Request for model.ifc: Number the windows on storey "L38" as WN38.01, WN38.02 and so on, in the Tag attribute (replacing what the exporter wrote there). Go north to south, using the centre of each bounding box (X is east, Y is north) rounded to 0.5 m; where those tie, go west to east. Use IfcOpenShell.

First a look at what the model holds.

```python
import ifcopenshell
import ifcopenshell.util.element
import ifcopenshell.util.placement

model = ifcopenshell.open("model.ifc")
print(model.schema)
storey = next(s for s in model.by_type("IfcBuildingStorey") if s.Name == "L38")
windows = [e for e in ifcopenshell.util.element.get_decomposition(storey) if e.is_a("IfcWindow")]
for e in sorted(windows, key=lambda e: e.id()):
    origin = ifcopenshell.util.placement.get_local_placement(e.ObjectPlacement)[:3, 3]
    print(e.id(), e.Tag, e.Name, origin.round(2) + 0.0, sep=" | ")
```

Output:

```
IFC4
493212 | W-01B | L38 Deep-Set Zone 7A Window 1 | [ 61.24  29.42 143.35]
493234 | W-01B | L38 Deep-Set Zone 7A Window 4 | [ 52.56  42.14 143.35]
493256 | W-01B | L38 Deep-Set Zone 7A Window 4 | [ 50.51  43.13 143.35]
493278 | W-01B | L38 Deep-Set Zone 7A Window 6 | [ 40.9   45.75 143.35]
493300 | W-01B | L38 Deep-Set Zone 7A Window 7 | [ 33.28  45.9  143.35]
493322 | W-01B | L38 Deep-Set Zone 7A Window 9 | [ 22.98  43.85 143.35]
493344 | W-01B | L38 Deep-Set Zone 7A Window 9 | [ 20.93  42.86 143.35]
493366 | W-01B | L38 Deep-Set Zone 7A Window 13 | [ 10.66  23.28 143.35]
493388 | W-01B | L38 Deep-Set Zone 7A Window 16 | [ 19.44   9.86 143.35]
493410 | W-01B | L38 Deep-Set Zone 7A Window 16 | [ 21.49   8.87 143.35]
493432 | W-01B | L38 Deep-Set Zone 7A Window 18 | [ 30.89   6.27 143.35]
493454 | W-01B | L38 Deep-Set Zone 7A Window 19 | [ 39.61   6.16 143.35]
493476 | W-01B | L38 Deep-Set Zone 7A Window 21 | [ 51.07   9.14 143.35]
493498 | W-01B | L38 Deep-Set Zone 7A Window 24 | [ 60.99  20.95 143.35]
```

```python
import ifcopenshell
import ifcopenshell.geom
import ifcopenshell.util.element
import ifcopenshell.util.shape

model = ifcopenshell.open("model.ifc")
settings = ifcopenshell.geom.settings()
settings.set("use-world-coords", True)


def centre(element):
    shape = ifcopenshell.geom.create_shape(settings, element)
    return ifcopenshell.util.shape.get_bbox_centroid(shape.geometry)


storey = next(s for s in model.by_type("IfcBuildingStorey") if s.Name == "L38")
windows = [e for e in ifcopenshell.util.element.get_decomposition(storey) if e.is_a("IfcWindow")]

# Insertion points can sit at a corner or the storey origin, so sort by the geometry (in metres).
centres = {e: centre(e) for e in windows}
windows.sort(key=lambda e: (-round(centres[e][1] / 0.5), centres[e][0]))

for i, e in enumerate(windows, start=1):
    number = f"WN38.{i:02d}"
    e.Tag = number
    print(e.id(), number)

model.write("model-out.ifc")
```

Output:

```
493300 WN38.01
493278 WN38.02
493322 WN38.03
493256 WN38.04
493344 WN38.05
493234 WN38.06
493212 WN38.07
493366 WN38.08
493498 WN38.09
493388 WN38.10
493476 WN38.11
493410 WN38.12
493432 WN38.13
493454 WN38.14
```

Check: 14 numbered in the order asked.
